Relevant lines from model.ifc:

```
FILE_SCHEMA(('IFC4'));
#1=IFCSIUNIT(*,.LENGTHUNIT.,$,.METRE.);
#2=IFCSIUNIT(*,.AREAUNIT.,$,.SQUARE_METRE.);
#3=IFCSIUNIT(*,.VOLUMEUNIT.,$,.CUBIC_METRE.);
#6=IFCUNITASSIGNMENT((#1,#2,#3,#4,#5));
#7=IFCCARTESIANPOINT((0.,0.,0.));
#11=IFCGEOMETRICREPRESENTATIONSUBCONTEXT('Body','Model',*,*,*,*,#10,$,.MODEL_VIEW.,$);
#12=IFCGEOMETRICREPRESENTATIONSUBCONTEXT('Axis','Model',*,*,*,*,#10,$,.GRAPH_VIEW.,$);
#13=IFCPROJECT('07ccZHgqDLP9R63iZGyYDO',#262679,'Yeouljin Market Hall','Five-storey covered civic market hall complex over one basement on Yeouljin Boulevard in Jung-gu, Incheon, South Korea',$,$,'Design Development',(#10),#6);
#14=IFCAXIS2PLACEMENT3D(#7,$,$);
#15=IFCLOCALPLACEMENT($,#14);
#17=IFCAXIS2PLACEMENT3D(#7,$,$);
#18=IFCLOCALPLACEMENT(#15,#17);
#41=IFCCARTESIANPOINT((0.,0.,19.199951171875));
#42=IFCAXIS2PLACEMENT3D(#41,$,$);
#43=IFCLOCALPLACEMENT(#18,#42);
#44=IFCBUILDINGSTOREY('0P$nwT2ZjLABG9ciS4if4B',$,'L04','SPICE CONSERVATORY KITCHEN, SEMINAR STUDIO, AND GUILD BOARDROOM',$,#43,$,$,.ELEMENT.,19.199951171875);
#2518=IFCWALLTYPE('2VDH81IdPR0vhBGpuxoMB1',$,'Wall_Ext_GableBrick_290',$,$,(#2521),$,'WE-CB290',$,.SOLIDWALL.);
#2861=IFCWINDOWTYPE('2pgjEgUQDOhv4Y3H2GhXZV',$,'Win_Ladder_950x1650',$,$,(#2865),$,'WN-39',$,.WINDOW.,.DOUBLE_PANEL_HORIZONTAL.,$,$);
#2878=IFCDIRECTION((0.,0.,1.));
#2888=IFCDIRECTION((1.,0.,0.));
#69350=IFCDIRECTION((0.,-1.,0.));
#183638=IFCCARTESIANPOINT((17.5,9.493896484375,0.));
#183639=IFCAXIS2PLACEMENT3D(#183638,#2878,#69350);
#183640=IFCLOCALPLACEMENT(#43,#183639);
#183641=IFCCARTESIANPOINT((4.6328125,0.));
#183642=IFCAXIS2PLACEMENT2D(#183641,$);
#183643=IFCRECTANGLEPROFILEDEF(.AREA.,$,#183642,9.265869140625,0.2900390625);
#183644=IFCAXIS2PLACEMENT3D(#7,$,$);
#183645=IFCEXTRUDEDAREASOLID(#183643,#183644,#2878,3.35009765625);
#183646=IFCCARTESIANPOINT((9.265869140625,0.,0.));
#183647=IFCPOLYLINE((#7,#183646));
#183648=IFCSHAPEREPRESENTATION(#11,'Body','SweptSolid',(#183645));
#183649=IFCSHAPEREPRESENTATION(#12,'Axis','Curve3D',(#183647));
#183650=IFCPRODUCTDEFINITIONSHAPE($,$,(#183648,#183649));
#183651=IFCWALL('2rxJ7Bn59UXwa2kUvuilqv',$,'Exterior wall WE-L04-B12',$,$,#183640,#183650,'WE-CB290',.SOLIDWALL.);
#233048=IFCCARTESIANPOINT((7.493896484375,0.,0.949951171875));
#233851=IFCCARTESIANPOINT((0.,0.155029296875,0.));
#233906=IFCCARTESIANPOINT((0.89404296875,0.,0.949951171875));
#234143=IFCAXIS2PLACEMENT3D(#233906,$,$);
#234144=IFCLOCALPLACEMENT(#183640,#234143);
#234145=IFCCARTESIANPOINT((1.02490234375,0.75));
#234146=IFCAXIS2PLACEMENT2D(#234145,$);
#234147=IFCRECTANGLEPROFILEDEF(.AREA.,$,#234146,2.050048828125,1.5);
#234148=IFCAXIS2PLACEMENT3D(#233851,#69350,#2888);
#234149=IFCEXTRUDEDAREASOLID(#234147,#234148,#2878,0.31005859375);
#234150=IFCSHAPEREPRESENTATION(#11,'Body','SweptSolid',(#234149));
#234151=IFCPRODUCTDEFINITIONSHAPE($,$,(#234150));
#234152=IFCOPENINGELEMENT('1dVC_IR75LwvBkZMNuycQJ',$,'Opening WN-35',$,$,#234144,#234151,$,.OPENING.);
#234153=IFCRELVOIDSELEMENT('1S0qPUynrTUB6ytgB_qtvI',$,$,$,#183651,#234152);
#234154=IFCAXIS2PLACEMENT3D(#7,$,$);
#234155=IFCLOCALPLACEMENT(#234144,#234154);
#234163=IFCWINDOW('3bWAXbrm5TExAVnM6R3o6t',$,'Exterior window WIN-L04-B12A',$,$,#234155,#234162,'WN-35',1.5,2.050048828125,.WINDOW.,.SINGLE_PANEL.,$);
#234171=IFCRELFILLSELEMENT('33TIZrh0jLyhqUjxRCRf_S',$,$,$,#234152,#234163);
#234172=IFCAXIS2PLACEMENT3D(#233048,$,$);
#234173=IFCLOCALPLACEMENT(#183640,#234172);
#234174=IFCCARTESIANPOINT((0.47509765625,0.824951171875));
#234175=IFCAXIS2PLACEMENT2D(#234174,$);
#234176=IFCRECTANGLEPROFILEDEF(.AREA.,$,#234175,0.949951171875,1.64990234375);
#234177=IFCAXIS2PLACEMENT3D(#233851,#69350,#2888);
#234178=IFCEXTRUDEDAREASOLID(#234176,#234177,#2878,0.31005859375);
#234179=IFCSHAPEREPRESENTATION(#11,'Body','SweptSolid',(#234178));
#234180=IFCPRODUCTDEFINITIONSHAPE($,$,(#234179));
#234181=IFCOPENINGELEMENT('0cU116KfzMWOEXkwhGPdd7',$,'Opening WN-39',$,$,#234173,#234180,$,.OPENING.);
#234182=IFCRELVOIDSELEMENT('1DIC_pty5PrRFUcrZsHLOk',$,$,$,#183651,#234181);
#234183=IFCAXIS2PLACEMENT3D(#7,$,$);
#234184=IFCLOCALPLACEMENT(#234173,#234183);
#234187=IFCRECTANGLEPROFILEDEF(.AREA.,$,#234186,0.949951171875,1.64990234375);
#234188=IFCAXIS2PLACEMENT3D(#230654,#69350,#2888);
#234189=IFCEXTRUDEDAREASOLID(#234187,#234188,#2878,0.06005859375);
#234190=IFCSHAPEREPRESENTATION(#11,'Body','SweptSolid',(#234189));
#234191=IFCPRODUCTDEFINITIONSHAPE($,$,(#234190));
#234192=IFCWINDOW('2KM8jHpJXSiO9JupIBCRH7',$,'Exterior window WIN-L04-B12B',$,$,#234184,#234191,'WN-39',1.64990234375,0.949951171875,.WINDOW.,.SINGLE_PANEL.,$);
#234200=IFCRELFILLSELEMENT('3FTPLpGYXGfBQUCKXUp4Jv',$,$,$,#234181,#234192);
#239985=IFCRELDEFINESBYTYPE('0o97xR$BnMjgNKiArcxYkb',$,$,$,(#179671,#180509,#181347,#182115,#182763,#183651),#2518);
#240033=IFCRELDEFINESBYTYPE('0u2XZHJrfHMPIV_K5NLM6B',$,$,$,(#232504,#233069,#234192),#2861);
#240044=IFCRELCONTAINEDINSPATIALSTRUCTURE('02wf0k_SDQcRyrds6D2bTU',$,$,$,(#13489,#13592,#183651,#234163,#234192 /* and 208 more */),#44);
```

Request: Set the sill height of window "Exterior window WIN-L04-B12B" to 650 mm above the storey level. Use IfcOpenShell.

```python
import numpy as np
import ifcopenshell
import ifcopenshell.api.geometry
import ifcopenshell.geom
import ifcopenshell.util.element
import ifcopenshell.util.placement
import ifcopenshell.util.shape
import ifcopenshell.util.unit

model = ifcopenshell.open("model.ifc")
unit_scale = ifcopenshell.util.unit.calculate_unit_scale(model)

window = model.by_guid("2KM8jHpJXSiO9JupIBCRH7")
opening = window.FillsVoids[0].RelatingOpeningElement
storey = ifcopenshell.util.element.get_container(window, ifc_class="IfcBuildingStorey")
level = ifcopenshell.util.placement.get_local_placement(storey.ObjectPlacement)[2, 3]

# The opening's origin need not be at the sill, so measure its lowest point.
shape = ifcopenshell.geom.create_shape(ifcopenshell.geom.settings(), opening)
bottom = ifcopenshell.util.shape.get_shape_bottom_elevation(shape, shape.geometry) / unit_scale
dz = level + 0.65 / unit_scale - bottom

shift = np.array([0.0, 0.0, dz])
# The window is placed relative to its opening, so it follows when the opening moves.
matrix = ifcopenshell.util.placement.get_local_placement(opening.ObjectPlacement)
matrix[:3, 3] += shift
ifcopenshell.api.geometry.edit_object_placement(
    model, product=opening, matrix=matrix, is_si=False, should_transform_children=True
)

print(f"moved by {dz * unit_scale:+.3f} m")

model.write("model_edited.ifc")
```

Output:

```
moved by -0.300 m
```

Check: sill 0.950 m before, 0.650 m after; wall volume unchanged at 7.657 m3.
